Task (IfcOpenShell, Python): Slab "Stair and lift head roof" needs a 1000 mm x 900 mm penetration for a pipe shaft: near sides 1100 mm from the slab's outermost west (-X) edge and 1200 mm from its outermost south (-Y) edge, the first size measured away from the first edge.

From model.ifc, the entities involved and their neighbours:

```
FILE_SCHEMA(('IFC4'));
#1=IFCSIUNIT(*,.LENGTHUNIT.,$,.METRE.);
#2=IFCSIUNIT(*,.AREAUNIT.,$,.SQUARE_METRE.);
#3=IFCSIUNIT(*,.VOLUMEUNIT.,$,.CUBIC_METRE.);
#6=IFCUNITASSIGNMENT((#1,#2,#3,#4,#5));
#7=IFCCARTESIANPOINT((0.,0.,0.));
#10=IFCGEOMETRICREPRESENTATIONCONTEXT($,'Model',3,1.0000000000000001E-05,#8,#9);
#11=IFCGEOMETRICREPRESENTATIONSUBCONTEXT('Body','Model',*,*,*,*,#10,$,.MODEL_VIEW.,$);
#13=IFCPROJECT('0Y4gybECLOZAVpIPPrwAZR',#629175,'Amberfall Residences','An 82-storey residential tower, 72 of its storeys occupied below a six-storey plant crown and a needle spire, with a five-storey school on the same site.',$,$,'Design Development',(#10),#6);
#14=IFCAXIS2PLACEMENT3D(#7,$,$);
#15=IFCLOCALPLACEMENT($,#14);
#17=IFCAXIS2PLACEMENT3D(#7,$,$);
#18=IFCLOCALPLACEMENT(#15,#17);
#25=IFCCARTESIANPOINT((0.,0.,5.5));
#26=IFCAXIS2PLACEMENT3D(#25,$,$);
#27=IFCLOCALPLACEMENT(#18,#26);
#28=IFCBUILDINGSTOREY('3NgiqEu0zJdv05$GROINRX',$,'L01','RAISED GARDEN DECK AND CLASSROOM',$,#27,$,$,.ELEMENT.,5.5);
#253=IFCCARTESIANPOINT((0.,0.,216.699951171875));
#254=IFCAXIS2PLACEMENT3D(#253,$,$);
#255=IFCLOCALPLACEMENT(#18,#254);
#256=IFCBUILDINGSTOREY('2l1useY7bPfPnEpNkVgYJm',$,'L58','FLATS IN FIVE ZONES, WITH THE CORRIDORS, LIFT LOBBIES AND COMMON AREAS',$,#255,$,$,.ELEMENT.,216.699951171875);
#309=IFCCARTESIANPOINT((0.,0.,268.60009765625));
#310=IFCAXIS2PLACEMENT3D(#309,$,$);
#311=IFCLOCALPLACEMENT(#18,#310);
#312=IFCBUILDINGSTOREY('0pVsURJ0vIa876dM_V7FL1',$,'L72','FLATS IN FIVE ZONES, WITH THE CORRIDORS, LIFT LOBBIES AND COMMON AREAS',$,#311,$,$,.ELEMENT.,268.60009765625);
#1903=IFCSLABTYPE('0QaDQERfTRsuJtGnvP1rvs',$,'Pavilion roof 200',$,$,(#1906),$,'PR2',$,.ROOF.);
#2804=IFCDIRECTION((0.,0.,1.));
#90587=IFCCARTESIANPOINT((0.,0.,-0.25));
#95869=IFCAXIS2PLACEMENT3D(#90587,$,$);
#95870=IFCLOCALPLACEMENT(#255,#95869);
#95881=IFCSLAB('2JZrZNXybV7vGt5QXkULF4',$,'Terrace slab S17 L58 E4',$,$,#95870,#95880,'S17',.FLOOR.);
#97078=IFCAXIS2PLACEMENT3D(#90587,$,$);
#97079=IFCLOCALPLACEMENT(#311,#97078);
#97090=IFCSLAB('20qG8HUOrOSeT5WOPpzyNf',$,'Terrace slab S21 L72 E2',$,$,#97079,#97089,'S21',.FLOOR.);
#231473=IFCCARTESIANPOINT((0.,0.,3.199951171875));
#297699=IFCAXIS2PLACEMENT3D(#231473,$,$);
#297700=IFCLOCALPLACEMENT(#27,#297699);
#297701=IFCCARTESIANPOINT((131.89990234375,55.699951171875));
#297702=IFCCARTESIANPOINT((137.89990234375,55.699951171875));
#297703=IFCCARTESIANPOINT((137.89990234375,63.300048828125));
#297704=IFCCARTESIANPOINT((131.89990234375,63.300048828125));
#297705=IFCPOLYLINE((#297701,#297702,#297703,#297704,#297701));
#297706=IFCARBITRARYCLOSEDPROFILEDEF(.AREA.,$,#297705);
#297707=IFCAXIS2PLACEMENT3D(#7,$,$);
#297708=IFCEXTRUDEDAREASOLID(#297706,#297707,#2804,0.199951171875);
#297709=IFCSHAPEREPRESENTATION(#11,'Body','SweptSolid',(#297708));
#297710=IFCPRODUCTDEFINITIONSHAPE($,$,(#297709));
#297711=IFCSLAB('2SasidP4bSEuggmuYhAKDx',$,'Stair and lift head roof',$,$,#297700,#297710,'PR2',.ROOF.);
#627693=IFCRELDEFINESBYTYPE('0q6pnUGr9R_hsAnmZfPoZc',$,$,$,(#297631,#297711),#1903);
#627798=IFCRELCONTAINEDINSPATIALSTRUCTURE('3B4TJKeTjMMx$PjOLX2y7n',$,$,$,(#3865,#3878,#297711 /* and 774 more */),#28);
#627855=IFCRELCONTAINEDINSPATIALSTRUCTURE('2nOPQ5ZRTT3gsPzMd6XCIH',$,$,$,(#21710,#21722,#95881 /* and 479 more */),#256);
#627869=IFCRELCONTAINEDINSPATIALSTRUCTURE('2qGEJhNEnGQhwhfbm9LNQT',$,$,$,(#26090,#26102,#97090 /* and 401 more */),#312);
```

```python
import numpy as np
import ifcopenshell
import ifcopenshell.api.feature
import ifcopenshell.api.geometry
import ifcopenshell.api.root
import ifcopenshell.geom
import ifcopenshell.util.placement
import ifcopenshell.util.representation
import ifcopenshell.util.shape
import ifcopenshell.util.unit

model = ifcopenshell.open("model.ifc")
unit_scale = ifcopenshell.util.unit.calculate_unit_scale(model)
settings = ifcopenshell.geom.settings()


def volume(element):
    """Net volume in cubic metres, openings subtracted."""
    shape = ifcopenshell.geom.create_shape(settings, element)
    return ifcopenshell.util.shape.get_volume(shape.geometry)


slab = model.by_guid("2SasidP4bSEuggmuYhAKDx")
before = volume(slab)

# Extent in the slab's own axes, in metres. The edges named are its -X and -Y sides.
slab_shape = ifcopenshell.geom.create_shape(settings, slab)
vertices = ifcopenshell.util.shape.get_vertices(slab_shape.geometry)
x_min, y_min, bottom = vertices.min(axis=0)
top = vertices[:, 2].max()

opening = ifcopenshell.api.root.create_entity(model, ifc_class="IfcOpeningElement", name="Pipe shaft opening", predefined_type="OPENING")
context = ifcopenshell.util.representation.get_context(model, "Model", "Body", "MODEL_VIEW")
width, depth = 1, 0.9
outline = [(0.0, 0.0), (width, 0.0), (width, depth), (0.0, depth), (0.0, 0.0)]
# Overshoot both faces by 50 mm so the cut is clean.
shape = ifcopenshell.api.geometry.add_slab_representation(
    model, context=context, depth=top - bottom + 0.1, polyline=outline
)
ifcopenshell.api.geometry.assign_representation(model, product=opening, representation=shape)

matrix = ifcopenshell.util.placement.get_local_placement(slab.ObjectPlacement)
matrix[:, 3] = matrix @ np.append(np.array([x_min + 1.1, y_min + 1.2, bottom - 0.05]) / unit_scale, 1.0)
ifcopenshell.api.geometry.edit_object_placement(model, product=opening, matrix=matrix, is_si=False)
ifcopenshell.api.feature.add_feature(model, feature=opening, element=slab)

after = volume(slab)

print(f"slab volume {before:.3f} -> {after:.3f} m3")

model.write("model_v2.ifc")
```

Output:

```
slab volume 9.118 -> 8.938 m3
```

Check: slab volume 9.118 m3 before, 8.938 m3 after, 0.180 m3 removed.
